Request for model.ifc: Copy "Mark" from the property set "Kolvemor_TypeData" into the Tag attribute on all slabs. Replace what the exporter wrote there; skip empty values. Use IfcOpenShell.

First a look at what the model holds.

```python
import ifcopenshell
import ifcopenshell.util.element

model = ifcopenshell.open("model.ifc")
print(model.schema)
slabs = model.by_type("IfcSlab")
print(len(slabs), "slabs")
for e in slabs[:8]:
    source = ifcopenshell.util.element.get_pset(e, "Kolvemor_TypeData", "Mark")
    target = e.Tag
    print(e.id(), repr(source), repr(target), sep=" | ")
```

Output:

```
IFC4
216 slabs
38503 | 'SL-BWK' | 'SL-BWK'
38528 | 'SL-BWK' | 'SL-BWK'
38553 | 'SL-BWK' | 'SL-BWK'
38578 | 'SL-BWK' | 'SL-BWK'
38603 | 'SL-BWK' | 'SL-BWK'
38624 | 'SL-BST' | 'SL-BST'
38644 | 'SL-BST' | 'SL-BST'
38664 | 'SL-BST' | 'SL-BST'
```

```python
import ifcopenshell
import ifcopenshell.util.element

model = ifcopenshell.open("model.ifc")

count = 0
for e in model.by_type("IfcSlab"):
    value = ifcopenshell.util.element.get_pset(e, "Kolvemor_TypeData", "Mark")
    current = e.Tag
    if not value or not value.strip() or current == value:
        continue
    e.Tag = value
    count += 1

print(count, "slabs updated")

model.write("model-out.ifc")
```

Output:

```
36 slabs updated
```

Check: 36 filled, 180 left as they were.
